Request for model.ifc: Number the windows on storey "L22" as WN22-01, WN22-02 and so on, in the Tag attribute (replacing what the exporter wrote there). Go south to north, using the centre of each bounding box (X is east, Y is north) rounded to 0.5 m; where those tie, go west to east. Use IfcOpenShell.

First a look at what the model holds.

```python
import ifcopenshell
import ifcopenshell.util.element
import ifcopenshell.util.placement

model = ifcopenshell.open("model.ifc")
print(model.schema)
storey = next(s for s in model.by_type("IfcBuildingStorey") if s.Name == "L22")
windows = [e for e in ifcopenshell.util.element.get_decomposition(storey) if e.is_a("IfcWindow")]
for e in sorted(windows, key=lambda e: e.id()):
    origin = ifcopenshell.util.placement.get_local_placement(e.ObjectPlacement)[:3, 3]
    print(e.id(), e.Tag, e.Name, origin.round(2) + 0.0, sep=" | ")
```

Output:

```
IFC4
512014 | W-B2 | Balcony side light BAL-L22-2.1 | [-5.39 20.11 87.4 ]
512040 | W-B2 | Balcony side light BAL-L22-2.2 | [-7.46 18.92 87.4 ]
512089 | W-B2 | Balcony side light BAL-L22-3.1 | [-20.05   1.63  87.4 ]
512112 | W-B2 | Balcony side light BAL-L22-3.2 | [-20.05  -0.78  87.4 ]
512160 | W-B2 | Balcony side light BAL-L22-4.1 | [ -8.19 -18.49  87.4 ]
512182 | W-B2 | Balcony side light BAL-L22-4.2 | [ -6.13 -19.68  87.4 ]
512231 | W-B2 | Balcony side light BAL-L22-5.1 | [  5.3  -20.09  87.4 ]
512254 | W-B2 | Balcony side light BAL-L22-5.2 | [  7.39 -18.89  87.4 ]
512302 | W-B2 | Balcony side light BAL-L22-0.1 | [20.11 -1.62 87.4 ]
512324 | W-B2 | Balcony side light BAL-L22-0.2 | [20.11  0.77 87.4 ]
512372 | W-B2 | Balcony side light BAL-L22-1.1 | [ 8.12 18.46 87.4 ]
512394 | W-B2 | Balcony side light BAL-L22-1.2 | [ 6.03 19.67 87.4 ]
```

```python
import ifcopenshell
import ifcopenshell.geom
import ifcopenshell.util.element
import ifcopenshell.util.shape

model = ifcopenshell.open("model.ifc")
settings = ifcopenshell.geom.settings()
settings.set("use-world-coords", True)


def centre(element):
    shape = ifcopenshell.geom.create_shape(settings, element)
    return ifcopenshell.util.shape.get_bbox_centroid(shape.geometry)


storey = next(s for s in model.by_type("IfcBuildingStorey") if s.Name == "L22")
windows = [e for e in ifcopenshell.util.element.get_decomposition(storey) if e.is_a("IfcWindow")]

# Insertion points can sit at a corner or the storey origin, so sort by the geometry (in metres).
centres = {e: centre(e) for e in windows}
windows.sort(key=lambda e: (round(centres[e][1] / 0.5), centres[e][0]))

for i, e in enumerate(windows, start=1):
    number = f"WN22-{i:02d}"
    e.Tag = number
    print(e.id(), number)

model.write("model_rev.ifc")
```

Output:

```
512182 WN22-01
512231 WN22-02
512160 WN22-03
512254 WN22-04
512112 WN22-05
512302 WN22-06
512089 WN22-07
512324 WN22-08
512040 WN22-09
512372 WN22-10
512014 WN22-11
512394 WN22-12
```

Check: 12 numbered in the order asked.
